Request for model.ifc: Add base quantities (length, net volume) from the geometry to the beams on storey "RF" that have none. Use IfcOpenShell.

First a look at what the model holds.

```python
import ifcopenshell
import ifcopenshell.util.element
import ifcopenshell.util.unit

model = ifcopenshell.open("model.ifc")
print(model.schema)
for unit_type in ("LENGTHUNIT", "AREAUNIT", "VOLUMEUNIT"):
    print(unit_type, ifcopenshell.util.unit.calculate_unit_scale(model, unit_type))
storey = next(s for s in model.by_type("IfcBuildingStorey") if s.Name == "RF")
beams = [e for e in ifcopenshell.util.element.get_decomposition(storey) if e.is_a("IfcBeam")]
for e in sorted(beams, key=lambda e: e.id()):
    print(e.id(), e.is_a(), e.Name, list(ifcopenshell.util.element.get_psets(e, qtos_only=True)), sep=" | ")
```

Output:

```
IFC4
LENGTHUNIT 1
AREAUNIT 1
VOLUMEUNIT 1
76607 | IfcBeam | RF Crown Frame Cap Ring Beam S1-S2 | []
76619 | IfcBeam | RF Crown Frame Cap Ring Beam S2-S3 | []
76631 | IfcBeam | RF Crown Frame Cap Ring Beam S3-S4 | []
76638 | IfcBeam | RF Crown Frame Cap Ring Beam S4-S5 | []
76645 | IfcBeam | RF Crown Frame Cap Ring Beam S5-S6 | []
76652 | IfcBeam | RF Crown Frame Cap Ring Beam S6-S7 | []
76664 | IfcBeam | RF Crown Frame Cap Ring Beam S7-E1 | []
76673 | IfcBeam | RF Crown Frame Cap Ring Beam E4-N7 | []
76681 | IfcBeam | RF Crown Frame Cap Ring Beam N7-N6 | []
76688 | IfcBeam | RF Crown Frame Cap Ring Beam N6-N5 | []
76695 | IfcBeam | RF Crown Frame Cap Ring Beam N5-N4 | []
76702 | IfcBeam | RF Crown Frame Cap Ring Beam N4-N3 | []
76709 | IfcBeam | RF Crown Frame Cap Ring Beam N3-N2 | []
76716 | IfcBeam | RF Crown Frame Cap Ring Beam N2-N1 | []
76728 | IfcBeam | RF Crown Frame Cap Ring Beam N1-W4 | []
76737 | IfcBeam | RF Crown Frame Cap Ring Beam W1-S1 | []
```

```python
import ifcopenshell
import ifcopenshell.api.pset
import ifcopenshell.geom
import ifcopenshell.util.element
import ifcopenshell.util.shape
import ifcopenshell.util.unit

model = ifcopenshell.open("model.ifc")
unit_scale = ifcopenshell.util.unit.calculate_unit_scale(model)
volume_scale = ifcopenshell.util.unit.calculate_unit_scale(model, "VOLUMEUNIT")
settings = ifcopenshell.geom.settings()

storey = next(s for s in model.by_type("IfcBuildingStorey") if s.Name == "RF")
beams = [e for e in ifcopenshell.util.element.get_decomposition(storey) if e.is_a("IfcBeam")]

for e in sorted(beams, key=lambda e: e.id()):
    if ifcopenshell.util.element.get_psets(e, qtos_only=True, should_inherit=False):
        continue
    # Geometry comes back in metres, in the element's own axes.
    shape = ifcopenshell.geom.create_shape(settings, e)
    values = {
        "Length": ifcopenshell.util.shape.get_max_xyz(shape.geometry) / unit_scale,
        "NetVolume": ifcopenshell.util.shape.get_volume(shape.geometry) / volume_scale,
    }
    qto = ifcopenshell.api.pset.add_qto(model, product=e, name="Qto_BeamBaseQuantities")
    ifcopenshell.api.pset.edit_qto(model, qto=qto, properties=values)
    print(e.id(), {k: round(v, 3) for k, v in values.items()})

model.write("model_rev.ifc")
```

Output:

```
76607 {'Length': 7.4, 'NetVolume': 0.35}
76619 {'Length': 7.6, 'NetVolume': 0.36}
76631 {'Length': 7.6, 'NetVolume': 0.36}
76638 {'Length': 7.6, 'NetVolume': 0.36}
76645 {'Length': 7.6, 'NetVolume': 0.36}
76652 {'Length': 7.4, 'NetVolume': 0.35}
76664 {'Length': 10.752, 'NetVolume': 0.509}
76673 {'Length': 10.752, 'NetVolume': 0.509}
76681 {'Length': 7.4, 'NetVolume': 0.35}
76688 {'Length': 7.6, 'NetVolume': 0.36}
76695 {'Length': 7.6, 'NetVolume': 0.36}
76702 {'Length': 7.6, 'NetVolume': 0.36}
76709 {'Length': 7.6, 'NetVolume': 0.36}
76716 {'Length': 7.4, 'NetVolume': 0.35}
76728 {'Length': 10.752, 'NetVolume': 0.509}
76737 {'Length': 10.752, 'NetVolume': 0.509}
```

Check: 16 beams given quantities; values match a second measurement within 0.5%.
